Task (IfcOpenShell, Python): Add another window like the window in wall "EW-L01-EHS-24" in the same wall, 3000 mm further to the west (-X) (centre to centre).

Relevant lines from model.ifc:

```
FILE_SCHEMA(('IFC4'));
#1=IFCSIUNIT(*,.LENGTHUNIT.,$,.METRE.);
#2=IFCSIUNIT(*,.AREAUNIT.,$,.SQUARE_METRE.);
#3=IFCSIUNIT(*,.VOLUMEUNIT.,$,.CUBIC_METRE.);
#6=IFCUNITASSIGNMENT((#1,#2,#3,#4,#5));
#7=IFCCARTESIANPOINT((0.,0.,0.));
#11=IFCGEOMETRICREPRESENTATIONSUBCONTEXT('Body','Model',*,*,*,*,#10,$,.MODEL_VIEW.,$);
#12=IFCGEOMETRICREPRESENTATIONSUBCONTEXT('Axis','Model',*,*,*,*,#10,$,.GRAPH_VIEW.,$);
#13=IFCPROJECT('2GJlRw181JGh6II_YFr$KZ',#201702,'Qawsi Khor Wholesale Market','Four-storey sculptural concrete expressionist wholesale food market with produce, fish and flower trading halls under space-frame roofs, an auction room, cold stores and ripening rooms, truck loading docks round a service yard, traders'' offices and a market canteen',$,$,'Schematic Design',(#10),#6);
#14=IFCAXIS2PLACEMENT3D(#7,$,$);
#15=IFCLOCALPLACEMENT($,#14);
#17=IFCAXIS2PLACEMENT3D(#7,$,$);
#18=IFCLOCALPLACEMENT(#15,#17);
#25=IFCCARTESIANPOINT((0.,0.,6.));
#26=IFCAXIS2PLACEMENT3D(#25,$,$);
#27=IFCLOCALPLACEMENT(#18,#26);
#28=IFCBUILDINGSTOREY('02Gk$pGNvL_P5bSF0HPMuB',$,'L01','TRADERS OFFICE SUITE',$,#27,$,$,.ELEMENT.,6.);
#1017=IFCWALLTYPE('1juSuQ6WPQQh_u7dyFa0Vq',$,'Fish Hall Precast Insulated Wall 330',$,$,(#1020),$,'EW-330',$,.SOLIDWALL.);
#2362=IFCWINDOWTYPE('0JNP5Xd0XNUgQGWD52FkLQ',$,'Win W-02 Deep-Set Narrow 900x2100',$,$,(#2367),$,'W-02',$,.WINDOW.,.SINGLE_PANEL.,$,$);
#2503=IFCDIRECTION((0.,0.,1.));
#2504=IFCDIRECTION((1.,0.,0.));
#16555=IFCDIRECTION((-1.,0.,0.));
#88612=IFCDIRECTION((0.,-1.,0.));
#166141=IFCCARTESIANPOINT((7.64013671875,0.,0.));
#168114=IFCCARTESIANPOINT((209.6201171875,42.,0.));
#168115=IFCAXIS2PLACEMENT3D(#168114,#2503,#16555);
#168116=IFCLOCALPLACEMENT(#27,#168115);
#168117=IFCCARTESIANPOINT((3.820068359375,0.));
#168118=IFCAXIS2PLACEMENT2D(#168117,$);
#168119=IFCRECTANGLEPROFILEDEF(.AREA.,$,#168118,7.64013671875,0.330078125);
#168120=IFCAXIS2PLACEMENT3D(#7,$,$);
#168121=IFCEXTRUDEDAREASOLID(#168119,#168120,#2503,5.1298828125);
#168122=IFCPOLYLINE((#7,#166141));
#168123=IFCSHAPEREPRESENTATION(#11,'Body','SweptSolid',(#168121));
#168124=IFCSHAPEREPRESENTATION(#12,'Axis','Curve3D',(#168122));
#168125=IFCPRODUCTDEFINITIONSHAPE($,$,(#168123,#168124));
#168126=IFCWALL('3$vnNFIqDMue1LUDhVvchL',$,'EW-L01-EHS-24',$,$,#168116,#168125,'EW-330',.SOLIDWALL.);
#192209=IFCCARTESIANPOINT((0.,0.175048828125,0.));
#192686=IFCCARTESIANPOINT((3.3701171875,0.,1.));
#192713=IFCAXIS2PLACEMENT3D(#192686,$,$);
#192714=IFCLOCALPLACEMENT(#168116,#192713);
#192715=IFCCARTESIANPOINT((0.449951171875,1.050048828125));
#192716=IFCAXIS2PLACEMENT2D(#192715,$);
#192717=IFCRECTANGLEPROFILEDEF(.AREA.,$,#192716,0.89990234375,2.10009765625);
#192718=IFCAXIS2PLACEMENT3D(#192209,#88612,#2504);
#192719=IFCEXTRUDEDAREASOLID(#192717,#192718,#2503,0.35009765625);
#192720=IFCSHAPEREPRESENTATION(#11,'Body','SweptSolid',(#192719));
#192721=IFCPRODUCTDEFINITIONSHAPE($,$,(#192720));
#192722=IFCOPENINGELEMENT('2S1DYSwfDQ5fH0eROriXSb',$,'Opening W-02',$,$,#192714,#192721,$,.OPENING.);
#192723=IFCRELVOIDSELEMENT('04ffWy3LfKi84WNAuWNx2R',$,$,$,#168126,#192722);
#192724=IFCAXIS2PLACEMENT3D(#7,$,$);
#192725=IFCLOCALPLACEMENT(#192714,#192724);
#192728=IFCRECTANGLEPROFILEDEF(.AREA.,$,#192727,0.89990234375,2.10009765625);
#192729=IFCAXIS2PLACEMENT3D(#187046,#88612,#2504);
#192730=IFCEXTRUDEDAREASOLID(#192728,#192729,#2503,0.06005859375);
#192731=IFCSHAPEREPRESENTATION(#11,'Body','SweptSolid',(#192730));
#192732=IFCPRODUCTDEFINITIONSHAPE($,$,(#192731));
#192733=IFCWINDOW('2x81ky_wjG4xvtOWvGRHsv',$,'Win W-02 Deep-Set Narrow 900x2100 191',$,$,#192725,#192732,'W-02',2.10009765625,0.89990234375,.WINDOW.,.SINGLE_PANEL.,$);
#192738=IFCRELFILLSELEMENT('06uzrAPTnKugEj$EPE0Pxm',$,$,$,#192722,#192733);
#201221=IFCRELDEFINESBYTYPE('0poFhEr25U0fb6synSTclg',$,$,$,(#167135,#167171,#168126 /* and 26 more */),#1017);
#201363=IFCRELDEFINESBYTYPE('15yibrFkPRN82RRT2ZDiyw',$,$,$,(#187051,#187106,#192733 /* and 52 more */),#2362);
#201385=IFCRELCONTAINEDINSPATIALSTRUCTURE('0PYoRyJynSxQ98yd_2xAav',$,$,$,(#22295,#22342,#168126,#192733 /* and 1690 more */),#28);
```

```python
import ifcopenshell
import ifcopenshell.api.feature
import ifcopenshell.api.geometry
import ifcopenshell.api.root
import ifcopenshell.geom
import ifcopenshell.util.element
import ifcopenshell.util.placement
import ifcopenshell.util.shape

model = ifcopenshell.open("model.ifc")
settings = ifcopenshell.geom.settings()


def volume(element):
    """Net volume in cubic metres, openings subtracted."""
    shape = ifcopenshell.geom.create_shape(settings, element)
    return ifcopenshell.util.shape.get_volume(shape.geometry)


window = model.by_guid("2x81ky_wjG4xvtOWvGRHsv")
opening = window.FillsVoids[0].RelatingOpeningElement
wall = opening.VoidsElements[0].RelatingBuildingElement
before = volume(wall)
shift = ifcopenshell.util.placement.get_local_placement(wall.ObjectPlacement)[:3, 0] * 3.0

# copy_class copies the void relationship, type, container and properties, but no geometry.
new_opening = ifcopenshell.api.root.copy_class(model, product=opening)
new_opening.Representation = ifcopenshell.util.element.copy_deep(
    model, opening.Representation, exclude=["IfcGeometricRepresentationContext", "IfcRepresentationMap"]
)
new_window = ifcopenshell.api.root.copy_class(model, product=window)
new_window.Representation = ifcopenshell.util.element.copy_deep(
    model, window.Representation, exclude=["IfcGeometricRepresentationContext", "IfcRepresentationMap"]
)
new_window.Tag = None
ifcopenshell.api.feature.add_filling(model, opening=new_opening, element=new_window)

for old, new in ((opening, new_opening), (window, new_window)):
    matrix = ifcopenshell.util.placement.get_local_placement(old.ObjectPlacement)
    matrix[:3, 3] += shift
    ifcopenshell.api.geometry.edit_object_placement(model, product=new, matrix=matrix, is_si=False)

after = volume(wall)

print(f"wall volume {before:.3f} -> {after:.3f} m3")

model.write("model_edited.ifc")
```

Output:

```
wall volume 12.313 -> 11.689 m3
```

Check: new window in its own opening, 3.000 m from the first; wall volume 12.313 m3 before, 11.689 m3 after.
